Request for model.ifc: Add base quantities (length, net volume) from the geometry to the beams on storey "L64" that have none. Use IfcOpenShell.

First a look at what the model holds.

```python
import ifcopenshell
import ifcopenshell.util.element
import ifcopenshell.util.unit

model = ifcopenshell.open("model.ifc")
print(model.schema)
for unit_type in ("LENGTHUNIT", "AREAUNIT", "VOLUMEUNIT"):
    print(unit_type, ifcopenshell.util.unit.calculate_unit_scale(model, unit_type))
storey = next(s for s in model.by_type("IfcBuildingStorey") if s.Name == "L64")
beams = [e for e in ifcopenshell.util.element.get_decomposition(storey) if e.is_a("IfcBeam")]
for e in sorted(beams, key=lambda e: e.id()):
    print(e.id(), e.is_a(), e.Name, list(ifcopenshell.util.element.get_psets(e, qtos_only=True)), sep=" | ")
```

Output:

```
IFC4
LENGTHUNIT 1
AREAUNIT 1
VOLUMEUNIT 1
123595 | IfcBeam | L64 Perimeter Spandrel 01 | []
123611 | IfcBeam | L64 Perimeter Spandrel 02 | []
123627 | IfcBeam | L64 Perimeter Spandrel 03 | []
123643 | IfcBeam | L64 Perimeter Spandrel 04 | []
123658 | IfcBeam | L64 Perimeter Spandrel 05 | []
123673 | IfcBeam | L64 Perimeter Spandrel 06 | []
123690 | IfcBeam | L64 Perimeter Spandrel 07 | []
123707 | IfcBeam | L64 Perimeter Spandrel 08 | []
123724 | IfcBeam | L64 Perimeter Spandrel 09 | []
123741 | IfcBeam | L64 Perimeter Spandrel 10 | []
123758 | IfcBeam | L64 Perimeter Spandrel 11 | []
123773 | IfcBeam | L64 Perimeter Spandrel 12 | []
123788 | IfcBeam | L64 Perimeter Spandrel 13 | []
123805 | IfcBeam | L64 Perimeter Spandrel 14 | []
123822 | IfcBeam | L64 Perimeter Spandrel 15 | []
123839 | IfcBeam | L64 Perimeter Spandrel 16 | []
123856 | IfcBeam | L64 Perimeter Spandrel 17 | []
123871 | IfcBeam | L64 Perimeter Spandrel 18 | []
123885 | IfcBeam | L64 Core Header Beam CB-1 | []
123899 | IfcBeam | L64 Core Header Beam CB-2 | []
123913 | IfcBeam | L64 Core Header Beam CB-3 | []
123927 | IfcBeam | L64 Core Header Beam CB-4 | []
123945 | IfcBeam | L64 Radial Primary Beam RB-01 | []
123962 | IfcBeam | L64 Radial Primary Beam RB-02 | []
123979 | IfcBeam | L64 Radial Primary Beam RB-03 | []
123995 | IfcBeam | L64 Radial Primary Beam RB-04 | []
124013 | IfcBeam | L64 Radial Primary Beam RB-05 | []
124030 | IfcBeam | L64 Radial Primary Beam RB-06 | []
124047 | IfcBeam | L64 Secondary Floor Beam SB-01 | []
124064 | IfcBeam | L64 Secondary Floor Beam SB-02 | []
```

```python
import ifcopenshell
import ifcopenshell.api.pset
import ifcopenshell.geom
import ifcopenshell.util.element
import ifcopenshell.util.shape
import ifcopenshell.util.unit

model = ifcopenshell.open("model.ifc")
unit_scale = ifcopenshell.util.unit.calculate_unit_scale(model)
volume_scale = ifcopenshell.util.unit.calculate_unit_scale(model, "VOLUMEUNIT")
settings = ifcopenshell.geom.settings()

storey = next(s for s in model.by_type("IfcBuildingStorey") if s.Name == "L64")
beams = [e for e in ifcopenshell.util.element.get_decomposition(storey) if e.is_a("IfcBeam")]

for e in sorted(beams, key=lambda e: e.id()):
    if ifcopenshell.util.element.get_psets(e, qtos_only=True, should_inherit=False):
        continue
    # Geometry comes back in metres, in the element's own axes.
    shape = ifcopenshell.geom.create_shape(settings, e)
    values = {
        "Length": ifcopenshell.util.shape.get_max_xyz(shape.geometry) / unit_scale,
        "NetVolume": ifcopenshell.util.shape.get_volume(shape.geometry) / volume_scale,
    }
    qto = ifcopenshell.api.pset.add_qto(model, product=e, name="Qto_BeamBaseQuantities")
    ifcopenshell.api.pset.edit_qto(model, qto=qto, properties=values)
    print(e.id(), {k: round(v, 3) for k, v in values.items()})

model.write("model_updated.ifc")
```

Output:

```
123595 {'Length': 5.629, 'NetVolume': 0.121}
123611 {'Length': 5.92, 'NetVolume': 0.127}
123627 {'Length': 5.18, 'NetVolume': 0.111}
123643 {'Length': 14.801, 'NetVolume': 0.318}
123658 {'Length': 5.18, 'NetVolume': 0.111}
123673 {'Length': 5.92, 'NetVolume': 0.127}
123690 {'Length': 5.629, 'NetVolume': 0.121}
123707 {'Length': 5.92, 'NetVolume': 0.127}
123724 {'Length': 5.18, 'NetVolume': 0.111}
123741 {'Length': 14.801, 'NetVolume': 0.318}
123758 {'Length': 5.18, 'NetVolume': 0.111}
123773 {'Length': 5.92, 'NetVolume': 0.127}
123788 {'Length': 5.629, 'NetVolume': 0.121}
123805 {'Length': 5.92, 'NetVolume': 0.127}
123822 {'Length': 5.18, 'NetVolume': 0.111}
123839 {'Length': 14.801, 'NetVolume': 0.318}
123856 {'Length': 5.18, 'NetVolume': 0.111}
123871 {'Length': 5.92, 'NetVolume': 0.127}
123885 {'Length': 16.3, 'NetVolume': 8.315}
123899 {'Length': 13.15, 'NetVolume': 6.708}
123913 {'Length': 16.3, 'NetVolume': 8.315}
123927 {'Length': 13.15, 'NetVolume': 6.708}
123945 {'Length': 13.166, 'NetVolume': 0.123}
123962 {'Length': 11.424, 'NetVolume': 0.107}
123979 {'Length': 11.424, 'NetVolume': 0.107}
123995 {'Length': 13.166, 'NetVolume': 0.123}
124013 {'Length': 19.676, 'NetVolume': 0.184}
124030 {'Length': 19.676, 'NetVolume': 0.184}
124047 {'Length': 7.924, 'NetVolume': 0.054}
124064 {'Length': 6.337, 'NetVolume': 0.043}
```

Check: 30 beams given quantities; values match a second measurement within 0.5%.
